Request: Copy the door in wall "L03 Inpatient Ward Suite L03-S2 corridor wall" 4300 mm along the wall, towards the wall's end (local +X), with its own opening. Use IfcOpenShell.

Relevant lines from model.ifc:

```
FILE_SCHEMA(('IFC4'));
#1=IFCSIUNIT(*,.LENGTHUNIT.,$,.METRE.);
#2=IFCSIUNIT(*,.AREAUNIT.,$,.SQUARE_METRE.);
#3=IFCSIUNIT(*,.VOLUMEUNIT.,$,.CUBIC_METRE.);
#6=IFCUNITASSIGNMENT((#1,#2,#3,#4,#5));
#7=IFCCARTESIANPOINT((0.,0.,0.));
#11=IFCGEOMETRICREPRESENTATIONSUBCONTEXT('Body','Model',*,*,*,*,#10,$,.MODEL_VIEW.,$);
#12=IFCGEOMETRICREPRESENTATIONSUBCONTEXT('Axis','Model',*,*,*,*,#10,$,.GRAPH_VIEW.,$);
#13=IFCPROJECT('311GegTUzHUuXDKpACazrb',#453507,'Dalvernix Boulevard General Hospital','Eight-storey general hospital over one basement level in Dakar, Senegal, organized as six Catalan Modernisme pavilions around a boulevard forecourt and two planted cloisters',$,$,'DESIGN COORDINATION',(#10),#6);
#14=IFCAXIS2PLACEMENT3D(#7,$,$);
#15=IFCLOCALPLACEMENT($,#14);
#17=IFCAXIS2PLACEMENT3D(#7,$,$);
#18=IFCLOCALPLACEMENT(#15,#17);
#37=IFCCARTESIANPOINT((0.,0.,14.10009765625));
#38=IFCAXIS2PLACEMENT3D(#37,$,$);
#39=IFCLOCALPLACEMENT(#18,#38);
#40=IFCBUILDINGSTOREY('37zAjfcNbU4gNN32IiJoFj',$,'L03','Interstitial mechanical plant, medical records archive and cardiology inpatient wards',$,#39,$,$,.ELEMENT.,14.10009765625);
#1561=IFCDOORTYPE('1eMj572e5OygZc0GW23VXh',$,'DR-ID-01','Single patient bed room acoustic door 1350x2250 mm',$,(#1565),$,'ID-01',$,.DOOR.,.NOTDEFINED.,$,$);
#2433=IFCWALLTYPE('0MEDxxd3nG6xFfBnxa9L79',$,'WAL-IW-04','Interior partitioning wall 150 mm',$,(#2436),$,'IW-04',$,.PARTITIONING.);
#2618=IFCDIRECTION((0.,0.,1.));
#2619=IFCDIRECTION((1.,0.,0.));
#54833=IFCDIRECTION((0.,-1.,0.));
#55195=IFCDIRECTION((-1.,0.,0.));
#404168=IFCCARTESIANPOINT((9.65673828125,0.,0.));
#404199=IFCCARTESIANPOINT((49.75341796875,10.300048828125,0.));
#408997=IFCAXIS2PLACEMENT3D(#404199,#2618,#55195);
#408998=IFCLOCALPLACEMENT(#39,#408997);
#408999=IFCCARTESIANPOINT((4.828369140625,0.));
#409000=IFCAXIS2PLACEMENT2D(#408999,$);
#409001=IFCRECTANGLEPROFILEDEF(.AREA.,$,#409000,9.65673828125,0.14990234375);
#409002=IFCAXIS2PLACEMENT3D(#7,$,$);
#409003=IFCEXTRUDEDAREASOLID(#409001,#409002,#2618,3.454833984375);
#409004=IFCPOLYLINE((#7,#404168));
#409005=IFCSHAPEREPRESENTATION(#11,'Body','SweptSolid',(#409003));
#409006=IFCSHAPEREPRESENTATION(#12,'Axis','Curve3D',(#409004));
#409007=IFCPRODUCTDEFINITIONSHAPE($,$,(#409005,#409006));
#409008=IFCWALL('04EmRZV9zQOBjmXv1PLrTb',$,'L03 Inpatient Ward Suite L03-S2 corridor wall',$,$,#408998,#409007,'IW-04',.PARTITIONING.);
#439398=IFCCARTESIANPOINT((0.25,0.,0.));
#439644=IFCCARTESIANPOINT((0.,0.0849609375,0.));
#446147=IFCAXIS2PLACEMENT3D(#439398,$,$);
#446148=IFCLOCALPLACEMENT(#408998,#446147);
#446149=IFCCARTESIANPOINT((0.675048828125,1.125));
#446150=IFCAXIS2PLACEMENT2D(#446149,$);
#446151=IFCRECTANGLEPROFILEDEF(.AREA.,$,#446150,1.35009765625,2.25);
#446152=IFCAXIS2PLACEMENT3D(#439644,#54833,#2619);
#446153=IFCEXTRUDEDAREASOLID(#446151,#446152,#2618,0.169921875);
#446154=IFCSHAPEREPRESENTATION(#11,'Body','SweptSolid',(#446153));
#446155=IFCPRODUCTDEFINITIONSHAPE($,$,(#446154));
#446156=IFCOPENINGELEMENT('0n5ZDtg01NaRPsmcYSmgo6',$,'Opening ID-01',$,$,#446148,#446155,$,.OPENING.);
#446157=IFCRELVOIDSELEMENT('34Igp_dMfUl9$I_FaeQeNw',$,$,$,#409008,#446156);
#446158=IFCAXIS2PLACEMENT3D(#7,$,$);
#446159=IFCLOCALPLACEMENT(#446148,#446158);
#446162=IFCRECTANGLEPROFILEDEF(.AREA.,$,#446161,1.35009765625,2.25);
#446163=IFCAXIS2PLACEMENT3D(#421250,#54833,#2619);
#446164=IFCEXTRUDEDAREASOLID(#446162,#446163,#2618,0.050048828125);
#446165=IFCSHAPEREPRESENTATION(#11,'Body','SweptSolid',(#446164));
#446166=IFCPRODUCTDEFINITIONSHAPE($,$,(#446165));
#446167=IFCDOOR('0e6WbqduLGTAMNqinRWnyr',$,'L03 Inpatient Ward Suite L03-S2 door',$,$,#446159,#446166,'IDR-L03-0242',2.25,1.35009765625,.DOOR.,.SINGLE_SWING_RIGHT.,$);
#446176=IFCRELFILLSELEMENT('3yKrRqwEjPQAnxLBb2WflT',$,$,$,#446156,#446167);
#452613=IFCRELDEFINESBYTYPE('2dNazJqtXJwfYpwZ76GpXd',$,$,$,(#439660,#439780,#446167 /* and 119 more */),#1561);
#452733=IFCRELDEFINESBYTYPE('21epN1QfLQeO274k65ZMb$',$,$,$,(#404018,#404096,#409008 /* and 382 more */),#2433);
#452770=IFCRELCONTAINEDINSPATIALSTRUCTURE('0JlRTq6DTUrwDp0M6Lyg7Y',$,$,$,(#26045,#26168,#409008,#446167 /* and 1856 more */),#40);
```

```python
import ifcopenshell
import ifcopenshell.api.feature
import ifcopenshell.api.geometry
import ifcopenshell.api.root
import ifcopenshell.geom
import ifcopenshell.util.element
import ifcopenshell.util.placement
import ifcopenshell.util.shape
import ifcopenshell.util.unit

model = ifcopenshell.open("model.ifc")
unit_scale = ifcopenshell.util.unit.calculate_unit_scale(model)
settings = ifcopenshell.geom.settings()


def volume(element):
    """Net volume in cubic metres, openings subtracted."""
    shape = ifcopenshell.geom.create_shape(settings, element)
    return ifcopenshell.util.shape.get_volume(shape.geometry)


door = model.by_id(446167)
opening = door.FillsVoids[0].RelatingOpeningElement
wall = opening.VoidsElements[0].RelatingBuildingElement
before = volume(wall)
shift = ifcopenshell.util.placement.get_local_placement(wall.ObjectPlacement)[:3, 0] * 4.3 / unit_scale

# copy_class copies the void relationship, type, container and properties, but no geometry.
new_opening = ifcopenshell.api.root.copy_class(model, product=opening)
new_opening.Representation = ifcopenshell.util.element.copy_deep(
    model, opening.Representation, exclude=["IfcGeometricRepresentationContext", "IfcRepresentationMap"]
)
new_door = ifcopenshell.api.root.copy_class(model, product=door)
new_door.Representation = ifcopenshell.util.element.copy_deep(
    model, door.Representation, exclude=["IfcGeometricRepresentationContext", "IfcRepresentationMap"]
)
new_door.Tag = None
ifcopenshell.api.feature.add_filling(model, opening=new_opening, element=new_door)

for old, new in ((opening, new_opening), (door, new_door)):
    matrix = ifcopenshell.util.placement.get_local_placement(old.ObjectPlacement)
    matrix[:3, 3] += shift
    ifcopenshell.api.geometry.edit_object_placement(model, product=new, matrix=matrix, is_si=False)

after = volume(wall)

print(f"wall volume {before:.3f} -> {after:.3f} m3")

model.write("model_v2.ifc")
```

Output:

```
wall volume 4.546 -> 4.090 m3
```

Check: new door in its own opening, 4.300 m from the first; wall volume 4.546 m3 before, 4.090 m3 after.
